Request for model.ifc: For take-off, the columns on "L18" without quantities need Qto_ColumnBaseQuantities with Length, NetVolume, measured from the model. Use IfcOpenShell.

First a look at what the model holds.

```python
import ifcopenshell
import ifcopenshell.util.element
import ifcopenshell.util.unit

model = ifcopenshell.open("model.ifc")
print(model.schema)
for unit_type in ("LENGTHUNIT", "AREAUNIT", "VOLUMEUNIT"):
    print(unit_type, ifcopenshell.util.unit.calculate_unit_scale(model, unit_type))
storey = next(s for s in model.by_type("IfcBuildingStorey") if s.Name == "L18")
columns = [e for e in ifcopenshell.util.element.get_decomposition(storey) if e.is_a("IfcColumn")]
for e in sorted(columns, key=lambda e: e.id()):
    print(e.id(), e.is_a(), e.Name, list(ifcopenshell.util.element.get_psets(e, qtos_only=True)), sep=" | ")
```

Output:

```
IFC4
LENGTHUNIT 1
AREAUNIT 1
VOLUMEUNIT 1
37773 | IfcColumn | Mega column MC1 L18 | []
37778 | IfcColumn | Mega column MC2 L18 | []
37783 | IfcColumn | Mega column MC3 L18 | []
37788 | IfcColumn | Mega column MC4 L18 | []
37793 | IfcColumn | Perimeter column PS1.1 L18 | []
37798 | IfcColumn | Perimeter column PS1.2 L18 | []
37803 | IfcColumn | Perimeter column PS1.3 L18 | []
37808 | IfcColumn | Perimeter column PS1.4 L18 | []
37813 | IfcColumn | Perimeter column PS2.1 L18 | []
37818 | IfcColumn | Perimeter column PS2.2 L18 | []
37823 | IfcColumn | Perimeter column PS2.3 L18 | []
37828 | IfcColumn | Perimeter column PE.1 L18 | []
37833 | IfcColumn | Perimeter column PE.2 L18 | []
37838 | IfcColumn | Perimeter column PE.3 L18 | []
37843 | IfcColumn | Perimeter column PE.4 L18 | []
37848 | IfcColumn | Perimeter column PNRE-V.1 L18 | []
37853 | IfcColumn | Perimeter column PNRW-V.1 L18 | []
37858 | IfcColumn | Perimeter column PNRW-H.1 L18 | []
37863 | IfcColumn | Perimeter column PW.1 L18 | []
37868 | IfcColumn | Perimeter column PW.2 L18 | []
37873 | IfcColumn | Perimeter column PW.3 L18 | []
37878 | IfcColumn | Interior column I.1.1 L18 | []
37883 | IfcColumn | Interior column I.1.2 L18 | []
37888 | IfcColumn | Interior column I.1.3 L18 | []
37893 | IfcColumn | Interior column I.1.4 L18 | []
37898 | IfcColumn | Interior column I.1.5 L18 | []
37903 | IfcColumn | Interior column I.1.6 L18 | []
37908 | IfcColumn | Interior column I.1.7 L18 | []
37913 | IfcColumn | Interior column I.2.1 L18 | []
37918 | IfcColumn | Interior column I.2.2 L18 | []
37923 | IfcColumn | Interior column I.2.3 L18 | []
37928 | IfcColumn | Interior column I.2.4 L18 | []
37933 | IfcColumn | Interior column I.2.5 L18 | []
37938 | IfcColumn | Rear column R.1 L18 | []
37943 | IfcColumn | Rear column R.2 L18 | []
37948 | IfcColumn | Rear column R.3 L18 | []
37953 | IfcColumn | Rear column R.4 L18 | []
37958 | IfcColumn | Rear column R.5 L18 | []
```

```python
import ifcopenshell
import ifcopenshell.api.pset
import ifcopenshell.geom
import ifcopenshell.util.element
import ifcopenshell.util.shape
import ifcopenshell.util.unit

model = ifcopenshell.open("model.ifc")
unit_scale = ifcopenshell.util.unit.calculate_unit_scale(model)
volume_scale = ifcopenshell.util.unit.calculate_unit_scale(model, "VOLUMEUNIT")
settings = ifcopenshell.geom.settings()

storey = next(s for s in model.by_type("IfcBuildingStorey") if s.Name == "L18")
columns = [e for e in ifcopenshell.util.element.get_decomposition(storey) if e.is_a("IfcColumn")]

for e in sorted(columns, key=lambda e: e.id()):
    if ifcopenshell.util.element.get_psets(e, qtos_only=True, should_inherit=False):
        continue
    # Geometry comes back in metres, in the element's own axes.
    shape = ifcopenshell.geom.create_shape(settings, e)
    values = {
        "Length": ifcopenshell.util.shape.get_z(shape.geometry) / unit_scale,
        "NetVolume": ifcopenshell.util.shape.get_volume(shape.geometry) / volume_scale,
    }
    qto = ifcopenshell.api.pset.add_qto(model, product=e, name="Qto_ColumnBaseQuantities")
    ifcopenshell.api.pset.edit_qto(model, qto=qto, properties=values)
    print(e.id(), {k: round(v, 3) for k, v in values.items()})

model.write("model_v2.ifc")
```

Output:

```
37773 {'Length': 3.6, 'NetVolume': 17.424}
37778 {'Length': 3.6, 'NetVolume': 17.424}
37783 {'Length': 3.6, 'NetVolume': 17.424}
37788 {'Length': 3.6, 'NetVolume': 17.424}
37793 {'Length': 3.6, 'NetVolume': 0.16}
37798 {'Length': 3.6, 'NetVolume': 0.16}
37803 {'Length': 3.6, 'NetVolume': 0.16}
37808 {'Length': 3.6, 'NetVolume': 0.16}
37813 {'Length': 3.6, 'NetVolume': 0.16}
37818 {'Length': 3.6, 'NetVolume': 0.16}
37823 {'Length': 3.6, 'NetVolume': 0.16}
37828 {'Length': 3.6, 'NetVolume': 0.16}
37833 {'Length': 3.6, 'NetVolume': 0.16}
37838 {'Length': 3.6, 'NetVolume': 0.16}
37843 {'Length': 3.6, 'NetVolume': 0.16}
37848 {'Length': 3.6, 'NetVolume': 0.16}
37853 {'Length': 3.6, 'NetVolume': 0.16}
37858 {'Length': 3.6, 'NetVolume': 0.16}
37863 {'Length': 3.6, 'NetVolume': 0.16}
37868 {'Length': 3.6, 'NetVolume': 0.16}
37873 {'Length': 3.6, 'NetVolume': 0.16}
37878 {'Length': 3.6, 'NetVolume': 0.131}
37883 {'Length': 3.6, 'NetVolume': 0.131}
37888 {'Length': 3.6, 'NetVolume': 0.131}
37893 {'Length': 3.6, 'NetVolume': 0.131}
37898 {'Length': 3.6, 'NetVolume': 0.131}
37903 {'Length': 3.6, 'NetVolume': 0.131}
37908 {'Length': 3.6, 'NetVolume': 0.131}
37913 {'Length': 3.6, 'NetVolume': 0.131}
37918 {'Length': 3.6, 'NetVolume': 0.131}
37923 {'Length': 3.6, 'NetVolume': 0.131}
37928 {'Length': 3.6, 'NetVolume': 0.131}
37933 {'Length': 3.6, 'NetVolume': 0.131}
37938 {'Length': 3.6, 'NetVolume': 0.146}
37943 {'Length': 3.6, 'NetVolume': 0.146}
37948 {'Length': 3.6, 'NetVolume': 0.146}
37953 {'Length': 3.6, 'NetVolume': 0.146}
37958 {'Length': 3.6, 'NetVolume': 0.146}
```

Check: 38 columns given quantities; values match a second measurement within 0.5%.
